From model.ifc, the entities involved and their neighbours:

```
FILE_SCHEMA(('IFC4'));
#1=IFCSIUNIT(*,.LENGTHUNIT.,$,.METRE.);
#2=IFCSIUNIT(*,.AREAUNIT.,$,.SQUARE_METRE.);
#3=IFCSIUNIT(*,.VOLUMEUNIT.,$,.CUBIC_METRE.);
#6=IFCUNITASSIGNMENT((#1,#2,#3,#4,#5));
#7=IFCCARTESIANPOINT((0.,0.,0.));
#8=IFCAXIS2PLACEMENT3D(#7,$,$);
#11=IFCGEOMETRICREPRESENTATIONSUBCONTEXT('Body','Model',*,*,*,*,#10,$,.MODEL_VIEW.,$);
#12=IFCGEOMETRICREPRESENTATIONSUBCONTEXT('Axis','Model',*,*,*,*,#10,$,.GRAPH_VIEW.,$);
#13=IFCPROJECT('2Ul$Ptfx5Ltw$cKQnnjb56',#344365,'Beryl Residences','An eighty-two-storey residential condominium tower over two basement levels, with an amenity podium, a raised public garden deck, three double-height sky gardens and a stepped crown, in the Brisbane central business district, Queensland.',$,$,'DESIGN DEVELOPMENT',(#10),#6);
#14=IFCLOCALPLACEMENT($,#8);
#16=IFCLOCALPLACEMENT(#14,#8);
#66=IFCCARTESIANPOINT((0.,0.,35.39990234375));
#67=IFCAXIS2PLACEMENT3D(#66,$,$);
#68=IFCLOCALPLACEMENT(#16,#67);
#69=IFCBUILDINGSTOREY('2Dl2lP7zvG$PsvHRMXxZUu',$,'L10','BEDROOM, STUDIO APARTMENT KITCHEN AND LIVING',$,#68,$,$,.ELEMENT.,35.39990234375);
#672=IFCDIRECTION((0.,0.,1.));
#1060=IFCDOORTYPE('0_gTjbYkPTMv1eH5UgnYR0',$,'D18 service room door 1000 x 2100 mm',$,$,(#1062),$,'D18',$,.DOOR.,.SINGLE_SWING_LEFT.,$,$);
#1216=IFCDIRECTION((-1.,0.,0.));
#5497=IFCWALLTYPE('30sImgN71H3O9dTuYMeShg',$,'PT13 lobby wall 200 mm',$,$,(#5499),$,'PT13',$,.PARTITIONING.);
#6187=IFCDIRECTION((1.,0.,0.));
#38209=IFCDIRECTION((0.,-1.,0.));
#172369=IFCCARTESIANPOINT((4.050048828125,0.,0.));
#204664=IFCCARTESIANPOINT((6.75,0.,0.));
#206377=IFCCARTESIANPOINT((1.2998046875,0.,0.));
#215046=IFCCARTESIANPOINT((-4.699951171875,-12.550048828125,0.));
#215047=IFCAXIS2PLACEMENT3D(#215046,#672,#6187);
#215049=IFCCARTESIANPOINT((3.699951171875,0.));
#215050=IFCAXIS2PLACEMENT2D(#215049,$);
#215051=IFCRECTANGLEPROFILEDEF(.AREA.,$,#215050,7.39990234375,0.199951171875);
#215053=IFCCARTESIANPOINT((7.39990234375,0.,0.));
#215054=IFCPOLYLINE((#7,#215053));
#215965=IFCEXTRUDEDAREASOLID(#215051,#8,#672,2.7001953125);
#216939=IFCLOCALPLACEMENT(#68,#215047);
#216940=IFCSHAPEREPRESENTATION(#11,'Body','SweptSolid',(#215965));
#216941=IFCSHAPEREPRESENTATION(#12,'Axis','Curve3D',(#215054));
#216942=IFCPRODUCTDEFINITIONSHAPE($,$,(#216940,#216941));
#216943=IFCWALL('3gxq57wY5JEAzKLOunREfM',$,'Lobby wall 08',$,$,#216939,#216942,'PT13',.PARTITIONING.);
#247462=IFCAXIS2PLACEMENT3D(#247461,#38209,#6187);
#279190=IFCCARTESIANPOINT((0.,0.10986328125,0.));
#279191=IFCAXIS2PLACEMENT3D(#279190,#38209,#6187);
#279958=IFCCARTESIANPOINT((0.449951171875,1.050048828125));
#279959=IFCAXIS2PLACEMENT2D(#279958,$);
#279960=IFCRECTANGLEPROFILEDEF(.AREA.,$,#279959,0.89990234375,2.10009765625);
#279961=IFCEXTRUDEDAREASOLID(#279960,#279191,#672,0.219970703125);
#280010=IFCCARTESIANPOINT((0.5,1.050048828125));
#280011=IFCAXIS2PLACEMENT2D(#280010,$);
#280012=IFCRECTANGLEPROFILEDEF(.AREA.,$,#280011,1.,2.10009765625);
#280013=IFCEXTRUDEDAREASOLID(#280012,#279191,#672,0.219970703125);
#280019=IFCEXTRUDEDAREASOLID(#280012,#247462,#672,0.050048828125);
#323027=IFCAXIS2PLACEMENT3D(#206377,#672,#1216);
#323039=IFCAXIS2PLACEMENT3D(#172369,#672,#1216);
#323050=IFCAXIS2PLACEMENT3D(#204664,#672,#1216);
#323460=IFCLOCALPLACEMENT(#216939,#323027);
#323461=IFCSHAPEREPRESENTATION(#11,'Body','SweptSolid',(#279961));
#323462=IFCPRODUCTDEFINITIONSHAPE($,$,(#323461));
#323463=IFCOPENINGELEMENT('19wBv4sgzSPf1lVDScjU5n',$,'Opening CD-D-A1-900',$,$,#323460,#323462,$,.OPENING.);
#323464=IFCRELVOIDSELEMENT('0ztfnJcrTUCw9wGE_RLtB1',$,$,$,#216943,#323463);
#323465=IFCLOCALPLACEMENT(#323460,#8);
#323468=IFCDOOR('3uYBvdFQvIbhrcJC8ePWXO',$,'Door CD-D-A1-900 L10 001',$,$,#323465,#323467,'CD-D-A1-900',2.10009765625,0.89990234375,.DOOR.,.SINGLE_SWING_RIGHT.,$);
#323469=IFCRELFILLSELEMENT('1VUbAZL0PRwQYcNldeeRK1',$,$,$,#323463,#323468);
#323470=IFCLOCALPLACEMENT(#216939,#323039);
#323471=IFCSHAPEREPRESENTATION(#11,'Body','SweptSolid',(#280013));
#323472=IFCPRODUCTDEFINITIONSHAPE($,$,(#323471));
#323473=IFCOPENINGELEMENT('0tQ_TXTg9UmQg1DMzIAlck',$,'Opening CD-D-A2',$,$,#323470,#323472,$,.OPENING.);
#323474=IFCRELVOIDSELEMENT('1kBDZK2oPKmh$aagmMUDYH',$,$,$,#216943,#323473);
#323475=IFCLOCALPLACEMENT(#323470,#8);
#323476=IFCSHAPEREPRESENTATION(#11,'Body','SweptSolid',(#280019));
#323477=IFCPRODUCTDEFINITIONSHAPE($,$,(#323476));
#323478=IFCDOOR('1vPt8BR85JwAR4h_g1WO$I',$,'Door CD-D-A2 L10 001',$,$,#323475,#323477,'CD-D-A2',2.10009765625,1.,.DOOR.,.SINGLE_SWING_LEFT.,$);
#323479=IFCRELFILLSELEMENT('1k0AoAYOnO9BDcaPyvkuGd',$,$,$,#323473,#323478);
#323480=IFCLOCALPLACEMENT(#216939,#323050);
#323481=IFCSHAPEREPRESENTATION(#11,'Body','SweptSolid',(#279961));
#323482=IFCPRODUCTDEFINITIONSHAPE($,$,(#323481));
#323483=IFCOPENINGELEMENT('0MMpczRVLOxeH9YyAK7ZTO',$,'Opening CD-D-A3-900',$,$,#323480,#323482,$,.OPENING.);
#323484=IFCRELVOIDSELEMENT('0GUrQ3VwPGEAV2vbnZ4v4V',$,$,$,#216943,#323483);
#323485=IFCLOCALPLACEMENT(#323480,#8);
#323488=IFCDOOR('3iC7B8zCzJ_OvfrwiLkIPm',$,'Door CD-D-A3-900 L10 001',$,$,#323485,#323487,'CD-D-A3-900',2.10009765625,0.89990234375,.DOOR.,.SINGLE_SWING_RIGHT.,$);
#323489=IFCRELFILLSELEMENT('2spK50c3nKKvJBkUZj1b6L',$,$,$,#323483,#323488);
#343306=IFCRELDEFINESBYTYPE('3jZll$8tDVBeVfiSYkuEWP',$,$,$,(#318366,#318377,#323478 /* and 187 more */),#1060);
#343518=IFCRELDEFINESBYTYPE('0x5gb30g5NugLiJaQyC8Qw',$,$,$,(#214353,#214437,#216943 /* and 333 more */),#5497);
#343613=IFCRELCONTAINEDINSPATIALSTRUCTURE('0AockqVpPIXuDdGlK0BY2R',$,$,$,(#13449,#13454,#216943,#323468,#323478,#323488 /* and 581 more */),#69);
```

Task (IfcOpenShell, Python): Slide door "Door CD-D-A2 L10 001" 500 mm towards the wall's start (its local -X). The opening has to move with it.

```python
import ifcopenshell
import ifcopenshell.api.geometry
import ifcopenshell.util.placement
import ifcopenshell.util.unit

model = ifcopenshell.open("model.ifc")
unit_scale = ifcopenshell.util.unit.calculate_unit_scale(model)

door = model.by_guid("1vPt8BR85JwAR4h_g1WO$I")
opening = door.FillsVoids[0].RelatingOpeningElement
wall = opening.VoidsElements[0].RelatingBuildingElement

wall_matrix = ifcopenshell.util.placement.get_local_placement(wall.ObjectPlacement)
shift = wall_matrix[:3, 0] * -0.5 / unit_scale
before = ifcopenshell.util.placement.get_local_placement(door.ObjectPlacement)[:3, 3].copy()

# The door is placed relative to its opening, so it follows when the opening moves.
matrix = ifcopenshell.util.placement.get_local_placement(opening.ObjectPlacement)
matrix[:3, 3] += shift
ifcopenshell.api.geometry.edit_object_placement(
    model, product=opening, matrix=matrix, is_si=False, should_transform_children=True
)

after = ifcopenshell.util.placement.get_local_placement(door.ObjectPlacement)[:3, 3]
print("door moved by", (after - before).round(3) + 0.0)

model.write("model_edited.ifc")
```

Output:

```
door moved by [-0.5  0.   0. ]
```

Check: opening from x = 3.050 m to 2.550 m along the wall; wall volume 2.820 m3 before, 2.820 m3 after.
